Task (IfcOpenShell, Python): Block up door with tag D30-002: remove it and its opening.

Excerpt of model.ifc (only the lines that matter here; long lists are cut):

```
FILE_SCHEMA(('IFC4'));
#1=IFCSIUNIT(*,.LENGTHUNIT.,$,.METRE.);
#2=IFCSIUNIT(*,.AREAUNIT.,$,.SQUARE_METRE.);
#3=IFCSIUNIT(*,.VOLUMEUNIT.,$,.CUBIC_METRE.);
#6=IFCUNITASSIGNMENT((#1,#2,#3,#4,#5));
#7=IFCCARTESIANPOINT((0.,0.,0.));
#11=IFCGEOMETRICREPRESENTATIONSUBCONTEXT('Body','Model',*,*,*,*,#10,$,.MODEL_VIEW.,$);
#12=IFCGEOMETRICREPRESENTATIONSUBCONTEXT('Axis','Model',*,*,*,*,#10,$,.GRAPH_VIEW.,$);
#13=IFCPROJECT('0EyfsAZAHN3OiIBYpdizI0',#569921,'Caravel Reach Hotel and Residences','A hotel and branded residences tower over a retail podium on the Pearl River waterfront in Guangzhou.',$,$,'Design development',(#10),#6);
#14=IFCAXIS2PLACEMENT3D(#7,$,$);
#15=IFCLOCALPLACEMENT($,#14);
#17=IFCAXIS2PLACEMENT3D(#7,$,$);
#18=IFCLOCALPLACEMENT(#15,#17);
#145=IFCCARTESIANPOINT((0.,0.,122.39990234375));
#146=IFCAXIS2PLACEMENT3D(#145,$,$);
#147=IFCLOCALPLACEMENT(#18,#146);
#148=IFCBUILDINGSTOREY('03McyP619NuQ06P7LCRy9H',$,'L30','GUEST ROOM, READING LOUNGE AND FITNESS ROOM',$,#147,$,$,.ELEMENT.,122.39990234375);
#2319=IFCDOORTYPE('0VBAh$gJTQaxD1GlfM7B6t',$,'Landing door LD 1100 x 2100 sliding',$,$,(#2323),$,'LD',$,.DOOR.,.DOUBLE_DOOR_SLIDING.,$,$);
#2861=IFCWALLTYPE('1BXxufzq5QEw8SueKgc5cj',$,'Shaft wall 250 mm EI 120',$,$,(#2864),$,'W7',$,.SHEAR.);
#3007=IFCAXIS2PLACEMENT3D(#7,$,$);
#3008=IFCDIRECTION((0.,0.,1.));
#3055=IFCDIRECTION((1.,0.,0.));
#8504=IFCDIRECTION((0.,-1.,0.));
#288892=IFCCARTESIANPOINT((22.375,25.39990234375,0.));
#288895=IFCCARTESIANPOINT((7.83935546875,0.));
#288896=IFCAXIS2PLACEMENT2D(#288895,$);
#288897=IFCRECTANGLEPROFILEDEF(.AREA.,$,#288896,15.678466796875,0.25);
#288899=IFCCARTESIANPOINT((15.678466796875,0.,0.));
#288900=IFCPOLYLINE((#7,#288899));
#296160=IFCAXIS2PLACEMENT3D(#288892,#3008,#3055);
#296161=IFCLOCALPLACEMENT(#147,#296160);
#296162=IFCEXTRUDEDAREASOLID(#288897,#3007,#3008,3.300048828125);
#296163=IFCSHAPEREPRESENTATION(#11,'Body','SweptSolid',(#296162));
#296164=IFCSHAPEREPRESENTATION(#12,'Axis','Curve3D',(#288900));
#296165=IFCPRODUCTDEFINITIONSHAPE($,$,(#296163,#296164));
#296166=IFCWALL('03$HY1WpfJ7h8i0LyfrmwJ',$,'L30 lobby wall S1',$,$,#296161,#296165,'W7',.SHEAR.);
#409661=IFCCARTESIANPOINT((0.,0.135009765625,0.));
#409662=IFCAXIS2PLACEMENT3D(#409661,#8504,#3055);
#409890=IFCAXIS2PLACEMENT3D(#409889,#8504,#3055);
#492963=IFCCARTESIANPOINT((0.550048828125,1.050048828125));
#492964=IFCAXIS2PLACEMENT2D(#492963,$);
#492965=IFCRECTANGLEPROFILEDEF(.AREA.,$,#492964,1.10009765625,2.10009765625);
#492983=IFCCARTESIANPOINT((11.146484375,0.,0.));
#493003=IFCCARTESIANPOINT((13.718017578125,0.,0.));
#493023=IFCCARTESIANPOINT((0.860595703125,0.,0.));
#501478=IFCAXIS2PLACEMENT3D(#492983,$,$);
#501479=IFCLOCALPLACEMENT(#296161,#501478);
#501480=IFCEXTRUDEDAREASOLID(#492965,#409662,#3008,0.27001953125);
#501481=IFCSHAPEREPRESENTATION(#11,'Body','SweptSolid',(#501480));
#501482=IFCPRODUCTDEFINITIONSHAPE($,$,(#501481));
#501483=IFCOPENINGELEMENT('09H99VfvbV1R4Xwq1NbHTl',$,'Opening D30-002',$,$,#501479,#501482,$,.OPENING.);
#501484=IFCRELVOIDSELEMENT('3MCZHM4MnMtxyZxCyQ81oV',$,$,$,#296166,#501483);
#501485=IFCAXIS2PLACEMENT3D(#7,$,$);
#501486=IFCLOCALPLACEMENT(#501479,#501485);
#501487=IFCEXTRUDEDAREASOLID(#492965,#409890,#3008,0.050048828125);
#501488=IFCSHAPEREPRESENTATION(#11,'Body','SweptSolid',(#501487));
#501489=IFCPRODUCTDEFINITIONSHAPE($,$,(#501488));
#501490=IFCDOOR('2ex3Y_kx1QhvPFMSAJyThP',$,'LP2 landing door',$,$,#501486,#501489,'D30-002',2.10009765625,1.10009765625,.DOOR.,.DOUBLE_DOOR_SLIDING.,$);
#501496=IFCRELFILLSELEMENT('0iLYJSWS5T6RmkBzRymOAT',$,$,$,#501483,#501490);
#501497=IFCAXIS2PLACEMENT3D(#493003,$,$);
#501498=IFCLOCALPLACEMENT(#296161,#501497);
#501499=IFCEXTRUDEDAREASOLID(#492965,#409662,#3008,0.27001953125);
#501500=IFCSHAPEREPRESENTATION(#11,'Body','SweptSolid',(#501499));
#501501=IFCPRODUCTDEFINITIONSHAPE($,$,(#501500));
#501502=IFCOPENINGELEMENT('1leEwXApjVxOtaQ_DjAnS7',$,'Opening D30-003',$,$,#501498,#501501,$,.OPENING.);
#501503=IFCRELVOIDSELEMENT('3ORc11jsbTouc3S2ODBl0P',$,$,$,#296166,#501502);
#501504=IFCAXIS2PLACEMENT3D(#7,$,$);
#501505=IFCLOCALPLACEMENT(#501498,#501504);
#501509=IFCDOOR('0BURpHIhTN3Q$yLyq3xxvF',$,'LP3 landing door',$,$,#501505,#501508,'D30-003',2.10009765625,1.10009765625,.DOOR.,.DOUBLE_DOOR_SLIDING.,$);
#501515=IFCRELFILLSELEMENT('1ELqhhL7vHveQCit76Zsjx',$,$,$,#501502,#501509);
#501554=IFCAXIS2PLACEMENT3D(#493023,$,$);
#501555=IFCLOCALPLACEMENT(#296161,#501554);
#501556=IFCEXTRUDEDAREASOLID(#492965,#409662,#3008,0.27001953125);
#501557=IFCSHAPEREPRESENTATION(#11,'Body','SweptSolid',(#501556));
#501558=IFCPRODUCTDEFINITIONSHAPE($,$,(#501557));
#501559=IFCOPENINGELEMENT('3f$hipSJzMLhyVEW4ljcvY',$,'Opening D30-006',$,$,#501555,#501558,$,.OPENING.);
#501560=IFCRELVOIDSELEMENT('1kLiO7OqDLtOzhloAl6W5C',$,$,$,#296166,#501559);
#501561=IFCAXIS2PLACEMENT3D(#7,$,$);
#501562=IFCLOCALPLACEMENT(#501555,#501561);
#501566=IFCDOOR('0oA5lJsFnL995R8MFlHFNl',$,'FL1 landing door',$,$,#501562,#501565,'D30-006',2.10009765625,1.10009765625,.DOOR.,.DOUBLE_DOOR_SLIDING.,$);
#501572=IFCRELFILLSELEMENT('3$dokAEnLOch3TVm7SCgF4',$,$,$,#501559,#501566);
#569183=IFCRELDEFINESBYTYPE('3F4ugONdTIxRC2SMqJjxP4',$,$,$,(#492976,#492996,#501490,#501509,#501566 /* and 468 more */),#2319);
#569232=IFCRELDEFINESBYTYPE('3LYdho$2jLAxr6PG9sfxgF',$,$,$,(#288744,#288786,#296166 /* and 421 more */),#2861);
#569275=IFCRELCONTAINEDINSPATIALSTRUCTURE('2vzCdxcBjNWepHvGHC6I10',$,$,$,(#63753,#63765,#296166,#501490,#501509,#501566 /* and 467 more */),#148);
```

```python
import ifcopenshell
import ifcopenshell.api.feature
import ifcopenshell.api.root
import ifcopenshell.geom
import ifcopenshell.util.shape

model = ifcopenshell.open("model.ifc")
settings = ifcopenshell.geom.settings()


def volume(element):
    """Net volume in cubic metres, openings subtracted."""
    shape = ifcopenshell.geom.create_shape(settings, element)
    return ifcopenshell.util.shape.get_volume(shape.geometry)


door = model.by_guid("2ex3Y_kx1QhvPFMSAJyThP")
opening = door.FillsVoids[0].RelatingOpeningElement
wall = opening.VoidsElements[0].RelatingBuildingElement
before = volume(wall)

ifcopenshell.api.root.remove_product(model, product=door)
ifcopenshell.api.feature.remove_feature(model, feature=opening)

after = volume(wall)

print(f"wall volume {before:.3f} -> {after:.3f} m3")

model.write("model_updated.ifc")
```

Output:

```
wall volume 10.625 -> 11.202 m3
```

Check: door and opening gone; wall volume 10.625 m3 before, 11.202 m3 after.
